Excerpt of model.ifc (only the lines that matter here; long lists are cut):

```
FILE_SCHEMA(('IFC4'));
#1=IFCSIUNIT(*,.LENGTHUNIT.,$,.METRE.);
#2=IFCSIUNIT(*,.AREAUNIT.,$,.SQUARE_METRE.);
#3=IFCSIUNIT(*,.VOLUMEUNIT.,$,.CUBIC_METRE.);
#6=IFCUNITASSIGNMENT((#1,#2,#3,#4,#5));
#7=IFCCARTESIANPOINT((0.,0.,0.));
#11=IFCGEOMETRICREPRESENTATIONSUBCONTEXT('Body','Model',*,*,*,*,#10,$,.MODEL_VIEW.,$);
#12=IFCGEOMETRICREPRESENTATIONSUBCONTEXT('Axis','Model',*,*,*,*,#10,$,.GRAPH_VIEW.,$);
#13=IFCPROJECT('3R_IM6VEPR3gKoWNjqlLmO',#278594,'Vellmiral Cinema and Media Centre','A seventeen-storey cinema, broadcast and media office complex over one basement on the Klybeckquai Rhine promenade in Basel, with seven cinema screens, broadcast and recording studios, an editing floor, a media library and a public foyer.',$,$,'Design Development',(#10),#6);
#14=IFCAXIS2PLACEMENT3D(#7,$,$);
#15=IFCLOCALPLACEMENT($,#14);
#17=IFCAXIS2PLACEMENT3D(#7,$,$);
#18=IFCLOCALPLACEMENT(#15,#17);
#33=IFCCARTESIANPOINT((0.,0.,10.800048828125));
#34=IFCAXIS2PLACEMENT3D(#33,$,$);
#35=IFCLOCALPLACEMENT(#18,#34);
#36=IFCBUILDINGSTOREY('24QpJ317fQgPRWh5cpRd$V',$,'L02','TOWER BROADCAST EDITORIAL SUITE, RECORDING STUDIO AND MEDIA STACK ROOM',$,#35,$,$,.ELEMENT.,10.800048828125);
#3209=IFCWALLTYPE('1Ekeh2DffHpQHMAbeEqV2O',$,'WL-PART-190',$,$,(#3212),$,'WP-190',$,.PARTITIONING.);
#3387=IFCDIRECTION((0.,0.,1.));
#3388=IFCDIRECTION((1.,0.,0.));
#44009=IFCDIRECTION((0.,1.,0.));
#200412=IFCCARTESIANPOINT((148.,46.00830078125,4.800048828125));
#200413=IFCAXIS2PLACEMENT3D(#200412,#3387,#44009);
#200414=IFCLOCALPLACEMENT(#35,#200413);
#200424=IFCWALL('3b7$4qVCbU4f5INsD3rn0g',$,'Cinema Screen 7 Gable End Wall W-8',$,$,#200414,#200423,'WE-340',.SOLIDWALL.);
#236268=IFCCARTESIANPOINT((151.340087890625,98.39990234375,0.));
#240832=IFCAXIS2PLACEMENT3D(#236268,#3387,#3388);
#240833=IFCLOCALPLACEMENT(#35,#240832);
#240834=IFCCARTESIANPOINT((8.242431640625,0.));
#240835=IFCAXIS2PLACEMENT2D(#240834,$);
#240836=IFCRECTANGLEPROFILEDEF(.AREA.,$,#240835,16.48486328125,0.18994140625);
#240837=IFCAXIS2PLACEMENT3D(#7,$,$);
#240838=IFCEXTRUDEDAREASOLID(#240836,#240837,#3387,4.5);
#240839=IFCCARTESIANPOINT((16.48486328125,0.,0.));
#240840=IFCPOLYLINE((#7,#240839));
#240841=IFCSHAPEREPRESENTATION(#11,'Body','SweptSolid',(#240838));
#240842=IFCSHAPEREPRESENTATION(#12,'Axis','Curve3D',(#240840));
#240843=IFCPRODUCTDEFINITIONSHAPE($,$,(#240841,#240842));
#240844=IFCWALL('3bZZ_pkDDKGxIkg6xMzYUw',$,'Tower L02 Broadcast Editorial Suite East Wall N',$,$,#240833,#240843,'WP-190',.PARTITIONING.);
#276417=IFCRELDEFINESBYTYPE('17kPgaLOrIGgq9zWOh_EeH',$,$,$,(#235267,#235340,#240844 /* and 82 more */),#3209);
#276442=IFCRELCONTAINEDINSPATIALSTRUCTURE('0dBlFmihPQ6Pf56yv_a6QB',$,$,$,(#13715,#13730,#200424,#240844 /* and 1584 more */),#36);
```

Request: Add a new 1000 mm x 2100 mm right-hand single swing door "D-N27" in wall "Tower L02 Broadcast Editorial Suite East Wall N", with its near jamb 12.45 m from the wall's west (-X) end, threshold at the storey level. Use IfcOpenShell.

```python
import numpy as np
import ifcopenshell
import ifcopenshell.api.feature
import ifcopenshell.api.geometry
import ifcopenshell.api.root
import ifcopenshell.api.spatial
import ifcopenshell.geom
import ifcopenshell.util.element
import ifcopenshell.util.placement
import ifcopenshell.util.representation
import ifcopenshell.util.shape
import ifcopenshell.util.unit

model = ifcopenshell.open("model.ifc")
unit_scale = ifcopenshell.util.unit.calculate_unit_scale(model)
settings = ifcopenshell.geom.settings()


def volume(element):
    """Net volume in cubic metres, openings subtracted."""
    shape = ifcopenshell.geom.create_shape(settings, element)
    return ifcopenshell.util.shape.get_volume(shape.geometry)


wall = model.by_guid("3bZZ_pkDDKGxIkg6xMzYUw")
storey = ifcopenshell.util.element.get_container(wall, ifc_class="IfcBuildingStorey")
context = ifcopenshell.util.representation.get_context(model, "Model", "Body", "MODEL_VIEW")
before = volume(wall)

width, height, from_end, sill = 1, 2.1, 12.45, 0.0  # metres

# The wall runs along its own X axis, and the end named is its -X end.
wall_shape = ifcopenshell.geom.create_shape(settings, wall)
x, y, z = ifcopenshell.util.shape.get_vertices(wall_shape.geometry).T
start = x.min() + from_end
face, thickness = float(y.min()), float(y.max() - y.min())
wall_matrix = ifcopenshell.util.placement.get_local_placement(wall.ObjectPlacement)
level = ifcopenshell.util.placement.get_local_placement(storey.ObjectPlacement)[2, 3]


def in_wall(x, y):
    """Placement at x, y metres in the wall's axes, at sill height."""
    matrix = wall_matrix.copy()
    matrix[:, 3] = wall_matrix @ np.array([x / unit_scale, y / unit_scale, 0.0, 1.0])
    matrix[2, 3] = level + sill / unit_scale
    return matrix


# Opening: a box that overshoots both wall faces by 50 mm.
opening = ifcopenshell.api.root.create_entity(model, ifc_class="IfcOpeningElement", predefined_type="OPENING")
box = ifcopenshell.api.geometry.add_wall_representation(
    model, context=context, length=width, height=height, thickness=thickness + 0.1
)
ifcopenshell.api.geometry.assign_representation(model, product=opening, representation=box)
ifcopenshell.api.geometry.edit_object_placement(model, product=opening, matrix=in_wall(start, face - 0.05), is_si=False)
ifcopenshell.api.feature.add_feature(model, feature=opening, element=wall)

door = ifcopenshell.api.root.create_entity(model, ifc_class="IfcDoor", name="D-N27", predefined_type="DOOR")
door.OverallWidth, door.OverallHeight = width / unit_scale, height / unit_scale
door.OperationType = "SINGLE_SWING_RIGHT"
body = ifcopenshell.api.geometry.add_door_representation(
    model,
    context=context,
    overall_width=door.OverallWidth,
    overall_height=door.OverallHeight,
    operation_type="SINGLE_SWING_RIGHT",
    lining_properties={"LiningDepth": thickness / unit_scale, "ThresholdDepth": thickness / unit_scale},
)
ifcopenshell.api.geometry.assign_representation(model, product=door, representation=body)
ifcopenshell.api.spatial.assign_container(model, products=[door], relating_structure=storey)
ifcopenshell.api.feature.add_filling(model, opening=opening, element=door)

# The lining spans the wall, so the door starts at the wall face.
ifcopenshell.api.geometry.edit_object_placement(model, product=door, matrix=in_wall(start, face), is_si=False)

after = volume(wall)

print(f"wall volume {before:.3f} -> {after:.3f} m3")

model.write("model_updated.ifc")
```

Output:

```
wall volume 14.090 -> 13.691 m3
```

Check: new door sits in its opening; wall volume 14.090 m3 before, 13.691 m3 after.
